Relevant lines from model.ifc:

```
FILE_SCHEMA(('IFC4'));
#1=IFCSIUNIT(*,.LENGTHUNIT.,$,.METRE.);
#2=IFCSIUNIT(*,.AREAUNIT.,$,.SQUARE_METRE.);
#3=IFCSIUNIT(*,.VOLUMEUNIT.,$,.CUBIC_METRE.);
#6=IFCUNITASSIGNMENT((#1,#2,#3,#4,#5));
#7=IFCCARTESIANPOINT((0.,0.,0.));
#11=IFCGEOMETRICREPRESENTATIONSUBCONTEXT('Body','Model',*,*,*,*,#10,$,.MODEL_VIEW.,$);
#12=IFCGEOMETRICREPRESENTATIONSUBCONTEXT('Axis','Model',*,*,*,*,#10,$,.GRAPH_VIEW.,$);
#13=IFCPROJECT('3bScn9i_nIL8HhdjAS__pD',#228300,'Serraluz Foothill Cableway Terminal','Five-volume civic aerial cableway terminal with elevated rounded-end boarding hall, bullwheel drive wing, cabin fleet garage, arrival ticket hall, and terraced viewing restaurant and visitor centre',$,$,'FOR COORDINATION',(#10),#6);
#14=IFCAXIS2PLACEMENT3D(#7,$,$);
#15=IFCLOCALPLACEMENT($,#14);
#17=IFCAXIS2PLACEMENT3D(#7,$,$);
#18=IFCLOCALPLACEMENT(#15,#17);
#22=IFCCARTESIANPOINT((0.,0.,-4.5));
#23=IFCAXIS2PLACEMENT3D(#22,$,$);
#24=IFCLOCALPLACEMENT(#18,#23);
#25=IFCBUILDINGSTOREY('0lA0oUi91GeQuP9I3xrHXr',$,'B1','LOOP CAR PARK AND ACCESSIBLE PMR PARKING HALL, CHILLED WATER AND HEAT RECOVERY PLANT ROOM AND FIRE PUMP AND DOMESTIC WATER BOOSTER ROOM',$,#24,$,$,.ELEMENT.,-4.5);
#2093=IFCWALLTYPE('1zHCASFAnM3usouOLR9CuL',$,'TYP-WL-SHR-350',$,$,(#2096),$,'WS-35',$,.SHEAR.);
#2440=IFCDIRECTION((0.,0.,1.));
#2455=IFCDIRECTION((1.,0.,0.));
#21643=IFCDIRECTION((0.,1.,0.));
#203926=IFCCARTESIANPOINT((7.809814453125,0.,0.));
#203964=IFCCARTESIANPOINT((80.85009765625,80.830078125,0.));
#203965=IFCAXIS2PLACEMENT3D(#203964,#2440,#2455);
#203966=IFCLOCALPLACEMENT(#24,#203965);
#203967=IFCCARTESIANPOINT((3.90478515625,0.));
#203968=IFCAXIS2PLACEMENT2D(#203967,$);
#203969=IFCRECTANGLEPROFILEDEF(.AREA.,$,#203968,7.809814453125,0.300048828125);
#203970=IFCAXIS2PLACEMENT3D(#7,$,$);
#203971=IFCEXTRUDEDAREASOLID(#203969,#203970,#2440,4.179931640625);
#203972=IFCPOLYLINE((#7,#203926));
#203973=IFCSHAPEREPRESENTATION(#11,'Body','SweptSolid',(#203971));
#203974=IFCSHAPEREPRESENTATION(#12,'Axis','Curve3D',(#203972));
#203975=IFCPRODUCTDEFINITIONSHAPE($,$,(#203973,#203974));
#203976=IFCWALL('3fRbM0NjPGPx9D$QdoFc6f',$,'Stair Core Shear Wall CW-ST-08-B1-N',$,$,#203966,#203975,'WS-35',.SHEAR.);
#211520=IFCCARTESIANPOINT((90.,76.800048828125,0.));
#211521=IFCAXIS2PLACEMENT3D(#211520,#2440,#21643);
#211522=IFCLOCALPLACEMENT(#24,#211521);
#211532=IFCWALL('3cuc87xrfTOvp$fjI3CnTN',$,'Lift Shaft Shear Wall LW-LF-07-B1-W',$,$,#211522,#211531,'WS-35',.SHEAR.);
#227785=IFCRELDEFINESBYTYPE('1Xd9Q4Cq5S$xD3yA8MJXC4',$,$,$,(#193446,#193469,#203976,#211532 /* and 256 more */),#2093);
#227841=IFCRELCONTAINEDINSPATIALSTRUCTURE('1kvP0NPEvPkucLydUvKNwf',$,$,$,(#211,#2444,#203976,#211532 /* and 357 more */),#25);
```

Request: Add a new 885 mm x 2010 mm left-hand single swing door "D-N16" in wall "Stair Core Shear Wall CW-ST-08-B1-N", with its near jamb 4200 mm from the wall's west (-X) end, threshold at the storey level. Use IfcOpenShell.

```python
import numpy as np
import ifcopenshell
import ifcopenshell.api.feature
import ifcopenshell.api.geometry
import ifcopenshell.api.root
import ifcopenshell.api.spatial
import ifcopenshell.geom
import ifcopenshell.util.element
import ifcopenshell.util.placement
import ifcopenshell.util.representation
import ifcopenshell.util.shape
import ifcopenshell.util.unit

model = ifcopenshell.open("model.ifc")
unit_scale = ifcopenshell.util.unit.calculate_unit_scale(model)
settings = ifcopenshell.geom.settings()


def volume(element):
    """Net volume in cubic metres, openings subtracted."""
    shape = ifcopenshell.geom.create_shape(settings, element)
    return ifcopenshell.util.shape.get_volume(shape.geometry)


wall = model.by_id(203976)
storey = ifcopenshell.util.element.get_container(wall, ifc_class="IfcBuildingStorey")
context = ifcopenshell.util.representation.get_context(model, "Model", "Body", "MODEL_VIEW")
before = volume(wall)

width, height, from_end, sill = 0.885, 2.01, 4.2, 0.0  # metres

# The wall runs along its own X axis, and the end named is its -X end.
wall_shape = ifcopenshell.geom.create_shape(settings, wall)
x, y, z = ifcopenshell.util.shape.get_vertices(wall_shape.geometry).T
start = x.min() + from_end
face, thickness = float(y.min()), float(y.max() - y.min())
wall_matrix = ifcopenshell.util.placement.get_local_placement(wall.ObjectPlacement)
level = ifcopenshell.util.placement.get_local_placement(storey.ObjectPlacement)[2, 3]


def in_wall(x, y):
    """Placement at x, y metres in the wall's axes, at sill height."""
    matrix = wall_matrix.copy()
    matrix[:, 3] = wall_matrix @ np.array([x / unit_scale, y / unit_scale, 0.0, 1.0])
    matrix[2, 3] = level + sill / unit_scale
    return matrix


# Opening: a box that overshoots both wall faces by 50 mm.
opening = ifcopenshell.api.root.create_entity(model, ifc_class="IfcOpeningElement", predefined_type="OPENING")
box = ifcopenshell.api.geometry.add_wall_representation(
    model, context=context, length=width, height=height, thickness=thickness + 0.1
)
ifcopenshell.api.geometry.assign_representation(model, product=opening, representation=box)
ifcopenshell.api.geometry.edit_object_placement(model, product=opening, matrix=in_wall(start, face - 0.05), is_si=False)
ifcopenshell.api.feature.add_feature(model, feature=opening, element=wall)

door = ifcopenshell.api.root.create_entity(model, ifc_class="IfcDoor", name="D-N16", predefined_type="DOOR")
door.OverallWidth, door.OverallHeight = width / unit_scale, height / unit_scale
door.OperationType = "SINGLE_SWING_LEFT"
body = ifcopenshell.api.geometry.add_door_representation(
    model,
    context=context,
    overall_width=door.OverallWidth,
    overall_height=door.OverallHeight,
    operation_type="SINGLE_SWING_LEFT",
    lining_properties={"LiningDepth": thickness / unit_scale, "ThresholdDepth": thickness / unit_scale},
)
ifcopenshell.api.geometry.assign_representation(model, product=door, representation=body)
ifcopenshell.api.spatial.assign_container(model, products=[door], relating_structure=storey)
ifcopenshell.api.feature.add_filling(model, opening=opening, element=door)

# The lining spans the wall, so the door starts at the wall face.
ifcopenshell.api.geometry.edit_object_placement(model, product=door, matrix=in_wall(start, face), is_si=False)

after = volume(wall)

print(f"wall volume {before:.3f} -> {after:.3f} m3")

model.write("model_v2.ifc")
```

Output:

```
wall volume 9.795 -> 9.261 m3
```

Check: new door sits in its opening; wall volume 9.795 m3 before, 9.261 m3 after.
